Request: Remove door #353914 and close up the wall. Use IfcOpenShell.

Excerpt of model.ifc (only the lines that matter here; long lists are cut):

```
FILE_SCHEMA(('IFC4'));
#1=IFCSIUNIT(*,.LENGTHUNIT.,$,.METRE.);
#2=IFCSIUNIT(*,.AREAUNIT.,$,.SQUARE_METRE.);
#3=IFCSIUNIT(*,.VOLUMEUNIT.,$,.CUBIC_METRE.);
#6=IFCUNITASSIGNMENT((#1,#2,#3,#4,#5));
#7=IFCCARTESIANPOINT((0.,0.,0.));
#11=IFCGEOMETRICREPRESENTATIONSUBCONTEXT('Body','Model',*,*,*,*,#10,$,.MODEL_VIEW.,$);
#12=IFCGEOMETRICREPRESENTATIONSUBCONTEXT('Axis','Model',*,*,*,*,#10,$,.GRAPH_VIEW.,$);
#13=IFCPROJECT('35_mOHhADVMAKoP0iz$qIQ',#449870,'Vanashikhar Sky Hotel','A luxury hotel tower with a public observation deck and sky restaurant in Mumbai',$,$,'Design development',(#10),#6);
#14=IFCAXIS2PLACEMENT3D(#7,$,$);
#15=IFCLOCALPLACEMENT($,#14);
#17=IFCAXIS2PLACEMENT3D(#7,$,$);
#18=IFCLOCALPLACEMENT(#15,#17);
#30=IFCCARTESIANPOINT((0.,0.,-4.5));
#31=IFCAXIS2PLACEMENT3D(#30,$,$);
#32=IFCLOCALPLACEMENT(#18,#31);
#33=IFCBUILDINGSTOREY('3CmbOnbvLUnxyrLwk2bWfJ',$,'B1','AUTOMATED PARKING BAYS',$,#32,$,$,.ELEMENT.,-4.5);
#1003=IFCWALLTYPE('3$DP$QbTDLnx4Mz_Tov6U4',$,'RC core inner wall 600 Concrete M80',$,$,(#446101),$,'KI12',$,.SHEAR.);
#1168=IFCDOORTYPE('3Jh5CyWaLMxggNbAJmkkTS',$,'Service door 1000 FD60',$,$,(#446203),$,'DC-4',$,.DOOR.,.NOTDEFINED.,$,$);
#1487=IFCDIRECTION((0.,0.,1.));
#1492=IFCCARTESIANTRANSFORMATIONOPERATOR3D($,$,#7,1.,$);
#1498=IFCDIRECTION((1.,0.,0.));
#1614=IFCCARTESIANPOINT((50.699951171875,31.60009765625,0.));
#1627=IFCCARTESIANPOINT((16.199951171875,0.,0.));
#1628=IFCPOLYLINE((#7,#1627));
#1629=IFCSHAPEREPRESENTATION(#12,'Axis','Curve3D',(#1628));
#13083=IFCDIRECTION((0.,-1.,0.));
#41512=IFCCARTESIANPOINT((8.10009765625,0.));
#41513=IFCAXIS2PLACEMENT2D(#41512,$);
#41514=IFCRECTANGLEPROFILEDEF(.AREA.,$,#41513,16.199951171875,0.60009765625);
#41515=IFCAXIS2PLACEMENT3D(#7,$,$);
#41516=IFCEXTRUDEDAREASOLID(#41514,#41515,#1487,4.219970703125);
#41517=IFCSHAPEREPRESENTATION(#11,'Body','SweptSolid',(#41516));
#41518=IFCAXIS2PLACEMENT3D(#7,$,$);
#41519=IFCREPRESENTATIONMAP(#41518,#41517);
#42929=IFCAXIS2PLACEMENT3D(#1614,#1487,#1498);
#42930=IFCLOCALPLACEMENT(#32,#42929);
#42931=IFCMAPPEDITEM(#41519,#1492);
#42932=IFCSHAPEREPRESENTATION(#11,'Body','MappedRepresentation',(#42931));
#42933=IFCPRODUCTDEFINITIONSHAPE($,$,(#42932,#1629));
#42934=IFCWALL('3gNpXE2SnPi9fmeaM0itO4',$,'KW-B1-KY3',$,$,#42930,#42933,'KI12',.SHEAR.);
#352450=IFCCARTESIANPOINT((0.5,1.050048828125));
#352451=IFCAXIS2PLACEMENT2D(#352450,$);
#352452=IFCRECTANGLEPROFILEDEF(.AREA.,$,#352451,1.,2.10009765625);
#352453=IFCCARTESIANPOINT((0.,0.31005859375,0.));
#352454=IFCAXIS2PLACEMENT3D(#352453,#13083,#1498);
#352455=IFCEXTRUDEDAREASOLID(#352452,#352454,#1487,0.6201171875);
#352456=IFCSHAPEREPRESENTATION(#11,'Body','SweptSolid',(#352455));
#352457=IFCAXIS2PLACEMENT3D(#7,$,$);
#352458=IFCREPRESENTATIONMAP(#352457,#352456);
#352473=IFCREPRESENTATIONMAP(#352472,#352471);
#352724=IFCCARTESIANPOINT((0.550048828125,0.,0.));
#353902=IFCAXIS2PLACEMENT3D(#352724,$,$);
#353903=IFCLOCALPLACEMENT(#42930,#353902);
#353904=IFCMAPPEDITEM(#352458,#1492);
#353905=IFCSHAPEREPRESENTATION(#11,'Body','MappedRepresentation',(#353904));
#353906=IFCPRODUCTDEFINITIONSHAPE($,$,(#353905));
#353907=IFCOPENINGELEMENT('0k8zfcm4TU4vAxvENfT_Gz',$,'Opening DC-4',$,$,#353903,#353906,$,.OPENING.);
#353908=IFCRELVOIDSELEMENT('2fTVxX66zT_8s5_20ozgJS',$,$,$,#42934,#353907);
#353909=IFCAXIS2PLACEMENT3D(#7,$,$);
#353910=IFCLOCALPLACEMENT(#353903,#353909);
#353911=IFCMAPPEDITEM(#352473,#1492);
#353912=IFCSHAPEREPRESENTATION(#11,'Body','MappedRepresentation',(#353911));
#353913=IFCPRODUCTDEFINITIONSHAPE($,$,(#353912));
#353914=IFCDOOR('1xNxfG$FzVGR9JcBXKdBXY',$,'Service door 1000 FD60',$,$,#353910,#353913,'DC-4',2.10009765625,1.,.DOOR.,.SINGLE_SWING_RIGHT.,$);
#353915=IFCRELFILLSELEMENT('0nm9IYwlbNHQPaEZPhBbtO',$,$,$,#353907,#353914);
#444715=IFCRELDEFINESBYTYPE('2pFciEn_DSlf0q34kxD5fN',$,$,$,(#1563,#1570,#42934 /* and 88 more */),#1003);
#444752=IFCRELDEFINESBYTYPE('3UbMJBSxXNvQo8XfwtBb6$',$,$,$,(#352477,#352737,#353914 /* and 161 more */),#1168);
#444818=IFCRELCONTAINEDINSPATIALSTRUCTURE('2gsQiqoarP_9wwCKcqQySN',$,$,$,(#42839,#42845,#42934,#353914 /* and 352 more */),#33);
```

```python
import ifcopenshell
import ifcopenshell.api.feature
import ifcopenshell.api.root
import ifcopenshell.geom
import ifcopenshell.util.shape

model = ifcopenshell.open("model.ifc")
settings = ifcopenshell.geom.settings()


def volume(element):
    """Net volume in cubic metres, openings subtracted."""
    shape = ifcopenshell.geom.create_shape(settings, element)
    return ifcopenshell.util.shape.get_volume(shape.geometry)


door = model.by_id(353914)
opening = door.FillsVoids[0].RelatingOpeningElement
wall = opening.VoidsElements[0].RelatingBuildingElement
before = volume(wall)

ifcopenshell.api.root.remove_product(model, product=door)
ifcopenshell.api.feature.remove_feature(model, feature=opening)

after = volume(wall)

print(f"wall volume {before:.3f} -> {after:.3f} m3")

model.write("model_v2.ifc")
```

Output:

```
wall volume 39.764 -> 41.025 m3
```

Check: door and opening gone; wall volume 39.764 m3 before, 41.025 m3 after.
